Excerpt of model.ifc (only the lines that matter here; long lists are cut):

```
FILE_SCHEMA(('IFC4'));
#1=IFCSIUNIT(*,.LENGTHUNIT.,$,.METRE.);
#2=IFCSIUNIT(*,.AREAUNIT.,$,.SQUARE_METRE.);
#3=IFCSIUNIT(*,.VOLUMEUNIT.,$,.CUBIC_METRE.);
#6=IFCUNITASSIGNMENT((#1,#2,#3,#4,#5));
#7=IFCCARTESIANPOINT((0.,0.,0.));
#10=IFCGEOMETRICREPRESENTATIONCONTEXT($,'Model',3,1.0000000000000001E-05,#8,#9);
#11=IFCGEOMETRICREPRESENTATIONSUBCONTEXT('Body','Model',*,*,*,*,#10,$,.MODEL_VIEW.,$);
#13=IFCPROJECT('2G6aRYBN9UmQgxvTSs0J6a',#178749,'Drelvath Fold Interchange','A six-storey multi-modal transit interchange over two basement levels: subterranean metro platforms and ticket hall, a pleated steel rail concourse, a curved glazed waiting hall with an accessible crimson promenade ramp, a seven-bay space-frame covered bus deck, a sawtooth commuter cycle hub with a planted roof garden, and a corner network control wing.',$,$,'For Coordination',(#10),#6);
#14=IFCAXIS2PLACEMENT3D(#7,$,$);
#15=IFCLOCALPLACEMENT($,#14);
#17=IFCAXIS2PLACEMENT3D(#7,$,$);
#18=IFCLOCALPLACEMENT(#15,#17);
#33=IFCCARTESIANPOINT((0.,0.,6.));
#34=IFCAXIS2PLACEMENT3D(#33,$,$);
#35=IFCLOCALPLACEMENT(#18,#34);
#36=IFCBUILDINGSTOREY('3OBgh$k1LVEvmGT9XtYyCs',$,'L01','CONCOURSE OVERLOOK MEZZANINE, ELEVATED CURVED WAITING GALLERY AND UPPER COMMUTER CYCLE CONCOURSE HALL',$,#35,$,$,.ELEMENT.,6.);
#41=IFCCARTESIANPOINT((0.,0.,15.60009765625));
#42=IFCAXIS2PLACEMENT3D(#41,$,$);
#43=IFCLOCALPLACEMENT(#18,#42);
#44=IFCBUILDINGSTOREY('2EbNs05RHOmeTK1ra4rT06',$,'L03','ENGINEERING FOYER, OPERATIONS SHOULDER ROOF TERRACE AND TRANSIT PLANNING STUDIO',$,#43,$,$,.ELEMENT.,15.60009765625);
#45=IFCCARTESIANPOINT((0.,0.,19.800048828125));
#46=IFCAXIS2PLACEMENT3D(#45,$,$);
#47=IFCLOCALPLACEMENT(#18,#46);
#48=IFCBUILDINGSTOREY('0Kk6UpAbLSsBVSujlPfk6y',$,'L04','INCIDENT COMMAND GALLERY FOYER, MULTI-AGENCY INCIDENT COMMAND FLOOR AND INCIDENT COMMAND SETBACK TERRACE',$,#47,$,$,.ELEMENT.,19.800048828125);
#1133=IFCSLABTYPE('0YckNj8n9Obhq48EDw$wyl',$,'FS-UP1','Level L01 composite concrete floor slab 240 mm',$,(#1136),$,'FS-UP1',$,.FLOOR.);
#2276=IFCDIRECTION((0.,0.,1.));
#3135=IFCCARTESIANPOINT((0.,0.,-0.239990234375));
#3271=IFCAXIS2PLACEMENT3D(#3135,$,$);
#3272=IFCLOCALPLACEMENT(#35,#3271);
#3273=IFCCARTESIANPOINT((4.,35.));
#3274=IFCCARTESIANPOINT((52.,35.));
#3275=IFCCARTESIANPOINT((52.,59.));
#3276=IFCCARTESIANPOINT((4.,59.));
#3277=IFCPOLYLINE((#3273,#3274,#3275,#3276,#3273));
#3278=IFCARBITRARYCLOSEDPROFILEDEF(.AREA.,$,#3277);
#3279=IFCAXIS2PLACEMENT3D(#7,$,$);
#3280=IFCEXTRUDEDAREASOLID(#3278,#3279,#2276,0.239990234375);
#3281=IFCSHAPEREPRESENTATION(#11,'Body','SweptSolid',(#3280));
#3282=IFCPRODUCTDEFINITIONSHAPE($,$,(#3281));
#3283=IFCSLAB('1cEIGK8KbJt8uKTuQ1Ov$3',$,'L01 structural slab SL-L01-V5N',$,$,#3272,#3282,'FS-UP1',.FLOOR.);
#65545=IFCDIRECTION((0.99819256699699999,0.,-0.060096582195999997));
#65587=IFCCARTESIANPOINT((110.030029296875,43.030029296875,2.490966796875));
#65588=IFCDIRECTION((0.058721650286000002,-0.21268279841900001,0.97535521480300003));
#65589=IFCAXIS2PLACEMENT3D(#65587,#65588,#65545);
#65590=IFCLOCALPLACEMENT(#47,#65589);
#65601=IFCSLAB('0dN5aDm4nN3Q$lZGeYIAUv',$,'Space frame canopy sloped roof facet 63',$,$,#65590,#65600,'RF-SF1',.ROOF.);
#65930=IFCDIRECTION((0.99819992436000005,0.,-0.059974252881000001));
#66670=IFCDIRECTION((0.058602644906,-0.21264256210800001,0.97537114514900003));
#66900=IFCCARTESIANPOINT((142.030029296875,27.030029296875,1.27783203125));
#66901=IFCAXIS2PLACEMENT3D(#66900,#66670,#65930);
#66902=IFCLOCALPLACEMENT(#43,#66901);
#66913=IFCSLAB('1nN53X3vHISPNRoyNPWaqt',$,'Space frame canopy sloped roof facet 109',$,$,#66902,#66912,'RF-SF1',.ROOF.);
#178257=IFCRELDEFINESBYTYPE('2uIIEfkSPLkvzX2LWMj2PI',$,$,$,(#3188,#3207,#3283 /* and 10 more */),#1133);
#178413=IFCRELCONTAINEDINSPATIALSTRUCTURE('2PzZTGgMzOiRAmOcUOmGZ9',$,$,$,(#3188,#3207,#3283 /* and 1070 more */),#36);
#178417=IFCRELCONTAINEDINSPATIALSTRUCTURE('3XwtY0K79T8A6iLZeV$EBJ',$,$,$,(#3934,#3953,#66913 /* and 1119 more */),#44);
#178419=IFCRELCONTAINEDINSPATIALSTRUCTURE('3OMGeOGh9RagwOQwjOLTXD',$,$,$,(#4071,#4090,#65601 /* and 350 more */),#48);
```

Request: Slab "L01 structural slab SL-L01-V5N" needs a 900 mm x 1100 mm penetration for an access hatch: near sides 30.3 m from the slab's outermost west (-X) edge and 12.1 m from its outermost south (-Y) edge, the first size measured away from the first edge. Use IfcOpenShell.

```python
import numpy as np
import ifcopenshell
import ifcopenshell.api.feature
import ifcopenshell.api.geometry
import ifcopenshell.api.root
import ifcopenshell.geom
import ifcopenshell.util.placement
import ifcopenshell.util.representation
import ifcopenshell.util.shape
import ifcopenshell.util.unit

model = ifcopenshell.open("model.ifc")
unit_scale = ifcopenshell.util.unit.calculate_unit_scale(model)
settings = ifcopenshell.geom.settings()


def volume(element):
    """Net volume in cubic metres, openings subtracted."""
    shape = ifcopenshell.geom.create_shape(settings, element)
    return ifcopenshell.util.shape.get_volume(shape.geometry)


slab = model.by_guid("1cEIGK8KbJt8uKTuQ1Ov$3")
before = volume(slab)

# Extent in the slab's own axes, in metres. The edges named are its -X and -Y sides.
slab_shape = ifcopenshell.geom.create_shape(settings, slab)
vertices = ifcopenshell.util.shape.get_vertices(slab_shape.geometry)
x_min, y_min, bottom = vertices.min(axis=0)
top = vertices[:, 2].max()

opening = ifcopenshell.api.root.create_entity(model, ifc_class="IfcOpeningElement", name="Access hatch opening", predefined_type="OPENING")
context = ifcopenshell.util.representation.get_context(model, "Model", "Body", "MODEL_VIEW")
width, depth = 0.9, 1.1
outline = [(0.0, 0.0), (width, 0.0), (width, depth), (0.0, depth), (0.0, 0.0)]
# Overshoot both faces by 50 mm so the cut is clean.
shape = ifcopenshell.api.geometry.add_slab_representation(
    model, context=context, depth=top - bottom + 0.1, polyline=outline
)
ifcopenshell.api.geometry.assign_representation(model, product=opening, representation=shape)

matrix = ifcopenshell.util.placement.get_local_placement(slab.ObjectPlacement)
matrix[:, 3] = matrix @ np.append(np.array([x_min + 30.3, y_min + 12.1, bottom - 0.05]) / unit_scale, 1.0)
ifcopenshell.api.geometry.edit_object_placement(model, product=opening, matrix=matrix, is_si=False)
ifcopenshell.api.feature.add_feature(model, feature=opening, element=slab)

after = volume(slab)

print(f"slab volume {before:.3f} -> {after:.3f} m3")

model.write("model_rev.ifc")
```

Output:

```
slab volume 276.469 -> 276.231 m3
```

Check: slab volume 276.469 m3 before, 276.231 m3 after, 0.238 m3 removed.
